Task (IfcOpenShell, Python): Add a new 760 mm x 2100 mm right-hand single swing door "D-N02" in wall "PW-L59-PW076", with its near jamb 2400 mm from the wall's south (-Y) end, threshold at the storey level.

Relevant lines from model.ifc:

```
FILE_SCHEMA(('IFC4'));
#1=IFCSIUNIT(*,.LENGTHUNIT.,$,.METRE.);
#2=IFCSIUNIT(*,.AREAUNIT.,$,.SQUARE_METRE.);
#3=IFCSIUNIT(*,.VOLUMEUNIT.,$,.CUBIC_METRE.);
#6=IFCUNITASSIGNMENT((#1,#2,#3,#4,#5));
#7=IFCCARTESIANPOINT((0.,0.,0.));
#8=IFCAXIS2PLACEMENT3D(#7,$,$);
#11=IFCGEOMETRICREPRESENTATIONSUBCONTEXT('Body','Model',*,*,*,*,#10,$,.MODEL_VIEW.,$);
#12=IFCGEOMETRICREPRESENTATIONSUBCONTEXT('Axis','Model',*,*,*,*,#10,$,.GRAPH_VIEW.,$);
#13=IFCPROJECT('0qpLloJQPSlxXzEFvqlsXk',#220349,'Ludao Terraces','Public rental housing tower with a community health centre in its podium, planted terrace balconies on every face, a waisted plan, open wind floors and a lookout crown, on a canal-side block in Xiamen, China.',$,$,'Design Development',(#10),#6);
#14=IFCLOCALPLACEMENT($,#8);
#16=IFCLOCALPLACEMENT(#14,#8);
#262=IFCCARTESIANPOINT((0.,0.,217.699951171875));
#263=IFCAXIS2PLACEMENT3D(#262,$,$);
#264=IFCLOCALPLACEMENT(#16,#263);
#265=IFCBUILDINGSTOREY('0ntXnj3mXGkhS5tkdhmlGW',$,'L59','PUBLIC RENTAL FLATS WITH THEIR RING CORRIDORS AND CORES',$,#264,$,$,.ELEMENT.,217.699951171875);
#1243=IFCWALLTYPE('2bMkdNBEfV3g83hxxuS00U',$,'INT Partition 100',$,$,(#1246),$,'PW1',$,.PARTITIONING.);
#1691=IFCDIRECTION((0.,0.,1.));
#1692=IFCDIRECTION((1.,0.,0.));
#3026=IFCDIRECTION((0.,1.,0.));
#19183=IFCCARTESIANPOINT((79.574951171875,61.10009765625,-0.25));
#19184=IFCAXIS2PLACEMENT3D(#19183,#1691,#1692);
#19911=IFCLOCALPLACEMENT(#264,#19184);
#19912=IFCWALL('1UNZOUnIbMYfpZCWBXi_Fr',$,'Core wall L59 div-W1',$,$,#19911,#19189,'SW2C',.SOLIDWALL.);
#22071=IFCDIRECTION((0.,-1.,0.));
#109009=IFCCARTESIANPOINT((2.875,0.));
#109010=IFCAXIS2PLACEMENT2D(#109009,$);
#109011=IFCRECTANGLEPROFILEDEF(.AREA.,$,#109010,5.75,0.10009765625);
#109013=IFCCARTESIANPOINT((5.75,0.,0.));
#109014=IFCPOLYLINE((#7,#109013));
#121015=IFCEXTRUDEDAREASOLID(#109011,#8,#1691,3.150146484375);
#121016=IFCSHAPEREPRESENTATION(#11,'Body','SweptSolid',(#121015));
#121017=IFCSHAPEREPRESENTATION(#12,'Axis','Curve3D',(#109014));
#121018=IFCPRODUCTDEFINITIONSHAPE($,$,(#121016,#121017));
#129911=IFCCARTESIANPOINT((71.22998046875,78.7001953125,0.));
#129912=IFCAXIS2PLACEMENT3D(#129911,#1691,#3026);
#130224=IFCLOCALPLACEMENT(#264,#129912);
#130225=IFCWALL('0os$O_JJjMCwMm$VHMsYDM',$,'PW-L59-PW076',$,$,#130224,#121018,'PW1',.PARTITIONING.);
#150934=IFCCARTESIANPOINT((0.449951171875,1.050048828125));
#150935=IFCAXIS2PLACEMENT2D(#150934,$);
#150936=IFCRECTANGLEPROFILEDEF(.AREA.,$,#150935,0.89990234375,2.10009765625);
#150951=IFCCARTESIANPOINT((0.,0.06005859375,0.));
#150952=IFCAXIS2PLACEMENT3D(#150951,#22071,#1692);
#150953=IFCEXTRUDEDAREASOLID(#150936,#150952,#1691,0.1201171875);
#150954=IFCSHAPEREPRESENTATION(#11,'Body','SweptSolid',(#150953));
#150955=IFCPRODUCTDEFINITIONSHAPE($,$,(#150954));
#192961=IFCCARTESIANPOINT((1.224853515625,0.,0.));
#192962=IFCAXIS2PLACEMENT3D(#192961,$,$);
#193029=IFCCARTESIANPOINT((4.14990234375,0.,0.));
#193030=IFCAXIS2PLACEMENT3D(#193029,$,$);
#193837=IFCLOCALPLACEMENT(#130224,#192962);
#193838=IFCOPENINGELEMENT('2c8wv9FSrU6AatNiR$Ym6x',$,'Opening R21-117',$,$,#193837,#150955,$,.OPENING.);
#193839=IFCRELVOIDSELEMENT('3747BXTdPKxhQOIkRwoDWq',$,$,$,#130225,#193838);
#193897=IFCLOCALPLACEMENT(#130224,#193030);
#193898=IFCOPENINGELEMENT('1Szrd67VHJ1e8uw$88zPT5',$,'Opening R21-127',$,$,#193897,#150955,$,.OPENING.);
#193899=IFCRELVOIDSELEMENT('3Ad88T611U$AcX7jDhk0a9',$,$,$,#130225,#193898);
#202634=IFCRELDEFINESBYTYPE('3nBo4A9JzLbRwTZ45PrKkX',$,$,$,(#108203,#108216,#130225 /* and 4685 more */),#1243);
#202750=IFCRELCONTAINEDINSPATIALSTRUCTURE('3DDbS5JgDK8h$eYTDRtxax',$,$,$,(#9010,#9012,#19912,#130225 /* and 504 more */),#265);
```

```python
import numpy as np
import ifcopenshell
import ifcopenshell.api.feature
import ifcopenshell.api.geometry
import ifcopenshell.api.root
import ifcopenshell.api.spatial
import ifcopenshell.geom
import ifcopenshell.util.element
import ifcopenshell.util.placement
import ifcopenshell.util.representation
import ifcopenshell.util.shape
import ifcopenshell.util.unit

model = ifcopenshell.open("model.ifc")
unit_scale = ifcopenshell.util.unit.calculate_unit_scale(model)
settings = ifcopenshell.geom.settings()


def volume(element):
    """Net volume in cubic metres, openings subtracted."""
    shape = ifcopenshell.geom.create_shape(settings, element)
    return ifcopenshell.util.shape.get_volume(shape.geometry)


wall = model.by_guid("0os$O_JJjMCwMm$VHMsYDM")
storey = ifcopenshell.util.element.get_container(wall, ifc_class="IfcBuildingStorey")
context = ifcopenshell.util.representation.get_context(model, "Model", "Body", "MODEL_VIEW")
before = volume(wall)

width, height, from_end, sill = 0.76, 2.1, 2.4, 0.0  # metres

# The wall runs along its own X axis, and the end named is its -X end.
wall_shape = ifcopenshell.geom.create_shape(settings, wall)
x, y, z = ifcopenshell.util.shape.get_vertices(wall_shape.geometry).T
start = x.min() + from_end
face, thickness = float(y.min()), float(y.max() - y.min())
wall_matrix = ifcopenshell.util.placement.get_local_placement(wall.ObjectPlacement)
level = ifcopenshell.util.placement.get_local_placement(storey.ObjectPlacement)[2, 3]


def in_wall(x, y):
    """Placement at x, y metres in the wall's axes, at sill height."""
    matrix = wall_matrix.copy()
    matrix[:, 3] = wall_matrix @ np.array([x / unit_scale, y / unit_scale, 0.0, 1.0])
    matrix[2, 3] = level + sill / unit_scale
    return matrix


# Opening: a box that overshoots both wall faces by 50 mm.
opening = ifcopenshell.api.root.create_entity(model, ifc_class="IfcOpeningElement", predefined_type="OPENING")
box = ifcopenshell.api.geometry.add_wall_representation(
    model, context=context, length=width, height=height, thickness=thickness + 0.1
)
ifcopenshell.api.geometry.assign_representation(model, product=opening, representation=box)
ifcopenshell.api.geometry.edit_object_placement(model, product=opening, matrix=in_wall(start, face - 0.05), is_si=False)
ifcopenshell.api.feature.add_feature(model, feature=opening, element=wall)

door = ifcopenshell.api.root.create_entity(model, ifc_class="IfcDoor", name="D-N02", predefined_type="DOOR")
door.OverallWidth, door.OverallHeight = width / unit_scale, height / unit_scale
door.OperationType = "SINGLE_SWING_RIGHT"
body = ifcopenshell.api.geometry.add_door_representation(
    model,
    context=context,
    overall_width=door.OverallWidth,
    overall_height=door.OverallHeight,
    operation_type="SINGLE_SWING_RIGHT",
    lining_properties={"LiningDepth": thickness / unit_scale, "ThresholdDepth": thickness / unit_scale},
)
ifcopenshell.api.geometry.assign_representation(model, product=door, representation=body)
ifcopenshell.api.spatial.assign_container(model, products=[door], relating_structure=storey)
ifcopenshell.api.feature.add_filling(model, opening=opening, element=door)

# The lining spans the wall, so the door starts at the wall face.
ifcopenshell.api.geometry.edit_object_placement(model, product=door, matrix=in_wall(start, face), is_si=False)

after = volume(wall)

print(f"wall volume {before:.3f} -> {after:.3f} m3")

model.write("model_rev.ifc")
```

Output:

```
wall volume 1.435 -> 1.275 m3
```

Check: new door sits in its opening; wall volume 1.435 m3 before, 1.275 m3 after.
